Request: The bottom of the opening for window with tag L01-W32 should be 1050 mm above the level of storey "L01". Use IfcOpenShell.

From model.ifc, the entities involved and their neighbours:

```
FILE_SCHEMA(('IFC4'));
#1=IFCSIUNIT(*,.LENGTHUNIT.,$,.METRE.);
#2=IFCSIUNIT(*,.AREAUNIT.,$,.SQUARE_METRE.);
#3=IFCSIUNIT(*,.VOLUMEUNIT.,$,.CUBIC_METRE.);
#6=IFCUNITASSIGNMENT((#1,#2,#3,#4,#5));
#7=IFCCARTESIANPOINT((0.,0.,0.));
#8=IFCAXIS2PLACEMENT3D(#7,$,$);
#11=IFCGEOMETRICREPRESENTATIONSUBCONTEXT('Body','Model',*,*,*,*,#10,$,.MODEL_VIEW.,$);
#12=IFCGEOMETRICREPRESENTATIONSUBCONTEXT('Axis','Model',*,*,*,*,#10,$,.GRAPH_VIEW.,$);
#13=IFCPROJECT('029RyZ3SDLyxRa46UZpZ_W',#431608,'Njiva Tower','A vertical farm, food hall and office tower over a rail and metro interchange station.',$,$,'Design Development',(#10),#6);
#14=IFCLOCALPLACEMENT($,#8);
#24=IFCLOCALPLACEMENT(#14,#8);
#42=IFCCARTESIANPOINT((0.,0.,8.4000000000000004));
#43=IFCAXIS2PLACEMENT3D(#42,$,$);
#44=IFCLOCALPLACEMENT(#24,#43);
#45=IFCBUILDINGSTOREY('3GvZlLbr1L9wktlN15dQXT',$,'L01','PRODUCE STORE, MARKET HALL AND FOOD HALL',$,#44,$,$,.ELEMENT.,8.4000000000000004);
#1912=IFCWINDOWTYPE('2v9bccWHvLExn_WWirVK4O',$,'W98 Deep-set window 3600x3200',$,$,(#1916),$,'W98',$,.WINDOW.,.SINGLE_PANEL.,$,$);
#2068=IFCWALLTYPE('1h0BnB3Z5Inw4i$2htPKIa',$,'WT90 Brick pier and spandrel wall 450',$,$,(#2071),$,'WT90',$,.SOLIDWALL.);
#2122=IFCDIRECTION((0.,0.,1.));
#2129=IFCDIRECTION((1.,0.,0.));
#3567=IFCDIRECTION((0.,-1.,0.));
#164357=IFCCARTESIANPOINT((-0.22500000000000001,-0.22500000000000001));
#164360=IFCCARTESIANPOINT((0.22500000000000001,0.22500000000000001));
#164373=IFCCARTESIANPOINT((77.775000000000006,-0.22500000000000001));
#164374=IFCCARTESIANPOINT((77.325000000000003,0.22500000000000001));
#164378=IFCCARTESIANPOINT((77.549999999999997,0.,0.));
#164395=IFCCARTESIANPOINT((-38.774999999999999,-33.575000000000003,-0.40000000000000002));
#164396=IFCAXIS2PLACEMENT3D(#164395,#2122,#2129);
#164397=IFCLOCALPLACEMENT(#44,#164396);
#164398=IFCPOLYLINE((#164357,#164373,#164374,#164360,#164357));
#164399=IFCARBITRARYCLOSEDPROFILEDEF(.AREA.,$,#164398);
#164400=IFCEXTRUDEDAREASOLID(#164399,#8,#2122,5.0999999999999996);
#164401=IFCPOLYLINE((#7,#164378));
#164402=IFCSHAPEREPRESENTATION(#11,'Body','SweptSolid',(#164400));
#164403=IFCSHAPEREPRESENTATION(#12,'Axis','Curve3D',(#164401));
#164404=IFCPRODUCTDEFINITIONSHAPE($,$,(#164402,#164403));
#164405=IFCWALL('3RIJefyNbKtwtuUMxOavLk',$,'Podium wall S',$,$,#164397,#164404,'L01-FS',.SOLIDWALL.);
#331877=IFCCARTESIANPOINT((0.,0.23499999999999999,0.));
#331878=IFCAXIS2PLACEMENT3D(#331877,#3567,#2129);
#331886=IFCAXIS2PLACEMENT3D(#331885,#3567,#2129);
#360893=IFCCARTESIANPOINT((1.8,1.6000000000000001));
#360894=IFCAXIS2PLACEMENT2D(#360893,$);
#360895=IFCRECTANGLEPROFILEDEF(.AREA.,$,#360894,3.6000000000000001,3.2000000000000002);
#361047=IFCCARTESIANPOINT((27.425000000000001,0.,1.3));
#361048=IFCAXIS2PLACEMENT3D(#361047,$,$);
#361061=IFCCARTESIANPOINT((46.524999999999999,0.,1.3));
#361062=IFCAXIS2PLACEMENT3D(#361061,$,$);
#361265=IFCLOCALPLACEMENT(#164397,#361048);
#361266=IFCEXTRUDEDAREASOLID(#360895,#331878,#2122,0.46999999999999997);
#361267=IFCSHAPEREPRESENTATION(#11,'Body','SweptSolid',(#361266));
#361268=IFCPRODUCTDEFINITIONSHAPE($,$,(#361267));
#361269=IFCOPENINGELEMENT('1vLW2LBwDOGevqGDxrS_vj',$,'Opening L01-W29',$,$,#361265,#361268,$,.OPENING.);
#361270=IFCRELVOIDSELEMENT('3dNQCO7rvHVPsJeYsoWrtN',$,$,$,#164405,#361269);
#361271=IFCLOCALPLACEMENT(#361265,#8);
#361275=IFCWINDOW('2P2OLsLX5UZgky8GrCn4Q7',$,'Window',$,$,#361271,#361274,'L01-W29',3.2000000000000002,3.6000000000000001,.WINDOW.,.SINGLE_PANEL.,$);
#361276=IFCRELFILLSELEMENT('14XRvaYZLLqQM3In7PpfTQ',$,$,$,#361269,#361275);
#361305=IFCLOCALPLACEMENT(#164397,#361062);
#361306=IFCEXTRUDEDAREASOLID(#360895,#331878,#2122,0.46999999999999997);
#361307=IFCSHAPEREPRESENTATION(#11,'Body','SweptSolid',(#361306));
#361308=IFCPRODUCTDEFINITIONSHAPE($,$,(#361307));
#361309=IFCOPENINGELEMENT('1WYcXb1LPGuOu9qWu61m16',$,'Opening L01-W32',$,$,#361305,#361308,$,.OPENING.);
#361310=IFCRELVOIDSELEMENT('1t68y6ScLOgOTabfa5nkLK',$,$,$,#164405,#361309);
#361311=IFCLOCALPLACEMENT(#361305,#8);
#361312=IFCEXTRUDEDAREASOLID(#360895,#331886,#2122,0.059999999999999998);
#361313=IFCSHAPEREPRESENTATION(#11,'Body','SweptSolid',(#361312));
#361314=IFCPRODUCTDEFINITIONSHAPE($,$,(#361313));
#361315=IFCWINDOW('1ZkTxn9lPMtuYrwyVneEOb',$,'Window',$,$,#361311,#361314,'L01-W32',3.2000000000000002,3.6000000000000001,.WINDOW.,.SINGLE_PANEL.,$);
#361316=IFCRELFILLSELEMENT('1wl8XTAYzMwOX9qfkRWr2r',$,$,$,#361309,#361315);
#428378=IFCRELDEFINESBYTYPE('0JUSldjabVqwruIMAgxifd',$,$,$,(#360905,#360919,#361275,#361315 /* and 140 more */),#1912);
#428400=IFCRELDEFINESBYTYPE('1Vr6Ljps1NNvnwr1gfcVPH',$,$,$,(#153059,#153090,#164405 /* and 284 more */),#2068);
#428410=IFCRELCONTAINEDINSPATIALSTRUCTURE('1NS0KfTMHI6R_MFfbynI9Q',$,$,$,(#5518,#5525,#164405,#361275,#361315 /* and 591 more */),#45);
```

```python
import numpy as np
import ifcopenshell
import ifcopenshell.api.geometry
import ifcopenshell.geom
import ifcopenshell.util.element
import ifcopenshell.util.placement
import ifcopenshell.util.shape
import ifcopenshell.util.unit

model = ifcopenshell.open("model.ifc")
unit_scale = ifcopenshell.util.unit.calculate_unit_scale(model)

window = model.by_guid("1ZkTxn9lPMtuYrwyVneEOb")
opening = window.FillsVoids[0].RelatingOpeningElement
storey = ifcopenshell.util.element.get_container(window, ifc_class="IfcBuildingStorey")
level = ifcopenshell.util.placement.get_local_placement(storey.ObjectPlacement)[2, 3]

# The opening's origin need not be at the sill, so measure its lowest point.
shape = ifcopenshell.geom.create_shape(ifcopenshell.geom.settings(), opening)
bottom = ifcopenshell.util.shape.get_shape_bottom_elevation(shape, shape.geometry) / unit_scale
dz = level + 1.05 / unit_scale - bottom

shift = np.array([0.0, 0.0, dz])
# The window is placed relative to its opening, so it follows when the opening moves.
matrix = ifcopenshell.util.placement.get_local_placement(opening.ObjectPlacement)
matrix[:3, 3] += shift
ifcopenshell.api.geometry.edit_object_placement(
    model, product=opening, matrix=matrix, is_si=False, should_transform_children=True
)

print(f"moved by {dz * unit_scale:+.3f} m")

model.write("model-out.ifc")
```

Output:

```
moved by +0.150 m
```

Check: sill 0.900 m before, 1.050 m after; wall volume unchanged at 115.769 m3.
